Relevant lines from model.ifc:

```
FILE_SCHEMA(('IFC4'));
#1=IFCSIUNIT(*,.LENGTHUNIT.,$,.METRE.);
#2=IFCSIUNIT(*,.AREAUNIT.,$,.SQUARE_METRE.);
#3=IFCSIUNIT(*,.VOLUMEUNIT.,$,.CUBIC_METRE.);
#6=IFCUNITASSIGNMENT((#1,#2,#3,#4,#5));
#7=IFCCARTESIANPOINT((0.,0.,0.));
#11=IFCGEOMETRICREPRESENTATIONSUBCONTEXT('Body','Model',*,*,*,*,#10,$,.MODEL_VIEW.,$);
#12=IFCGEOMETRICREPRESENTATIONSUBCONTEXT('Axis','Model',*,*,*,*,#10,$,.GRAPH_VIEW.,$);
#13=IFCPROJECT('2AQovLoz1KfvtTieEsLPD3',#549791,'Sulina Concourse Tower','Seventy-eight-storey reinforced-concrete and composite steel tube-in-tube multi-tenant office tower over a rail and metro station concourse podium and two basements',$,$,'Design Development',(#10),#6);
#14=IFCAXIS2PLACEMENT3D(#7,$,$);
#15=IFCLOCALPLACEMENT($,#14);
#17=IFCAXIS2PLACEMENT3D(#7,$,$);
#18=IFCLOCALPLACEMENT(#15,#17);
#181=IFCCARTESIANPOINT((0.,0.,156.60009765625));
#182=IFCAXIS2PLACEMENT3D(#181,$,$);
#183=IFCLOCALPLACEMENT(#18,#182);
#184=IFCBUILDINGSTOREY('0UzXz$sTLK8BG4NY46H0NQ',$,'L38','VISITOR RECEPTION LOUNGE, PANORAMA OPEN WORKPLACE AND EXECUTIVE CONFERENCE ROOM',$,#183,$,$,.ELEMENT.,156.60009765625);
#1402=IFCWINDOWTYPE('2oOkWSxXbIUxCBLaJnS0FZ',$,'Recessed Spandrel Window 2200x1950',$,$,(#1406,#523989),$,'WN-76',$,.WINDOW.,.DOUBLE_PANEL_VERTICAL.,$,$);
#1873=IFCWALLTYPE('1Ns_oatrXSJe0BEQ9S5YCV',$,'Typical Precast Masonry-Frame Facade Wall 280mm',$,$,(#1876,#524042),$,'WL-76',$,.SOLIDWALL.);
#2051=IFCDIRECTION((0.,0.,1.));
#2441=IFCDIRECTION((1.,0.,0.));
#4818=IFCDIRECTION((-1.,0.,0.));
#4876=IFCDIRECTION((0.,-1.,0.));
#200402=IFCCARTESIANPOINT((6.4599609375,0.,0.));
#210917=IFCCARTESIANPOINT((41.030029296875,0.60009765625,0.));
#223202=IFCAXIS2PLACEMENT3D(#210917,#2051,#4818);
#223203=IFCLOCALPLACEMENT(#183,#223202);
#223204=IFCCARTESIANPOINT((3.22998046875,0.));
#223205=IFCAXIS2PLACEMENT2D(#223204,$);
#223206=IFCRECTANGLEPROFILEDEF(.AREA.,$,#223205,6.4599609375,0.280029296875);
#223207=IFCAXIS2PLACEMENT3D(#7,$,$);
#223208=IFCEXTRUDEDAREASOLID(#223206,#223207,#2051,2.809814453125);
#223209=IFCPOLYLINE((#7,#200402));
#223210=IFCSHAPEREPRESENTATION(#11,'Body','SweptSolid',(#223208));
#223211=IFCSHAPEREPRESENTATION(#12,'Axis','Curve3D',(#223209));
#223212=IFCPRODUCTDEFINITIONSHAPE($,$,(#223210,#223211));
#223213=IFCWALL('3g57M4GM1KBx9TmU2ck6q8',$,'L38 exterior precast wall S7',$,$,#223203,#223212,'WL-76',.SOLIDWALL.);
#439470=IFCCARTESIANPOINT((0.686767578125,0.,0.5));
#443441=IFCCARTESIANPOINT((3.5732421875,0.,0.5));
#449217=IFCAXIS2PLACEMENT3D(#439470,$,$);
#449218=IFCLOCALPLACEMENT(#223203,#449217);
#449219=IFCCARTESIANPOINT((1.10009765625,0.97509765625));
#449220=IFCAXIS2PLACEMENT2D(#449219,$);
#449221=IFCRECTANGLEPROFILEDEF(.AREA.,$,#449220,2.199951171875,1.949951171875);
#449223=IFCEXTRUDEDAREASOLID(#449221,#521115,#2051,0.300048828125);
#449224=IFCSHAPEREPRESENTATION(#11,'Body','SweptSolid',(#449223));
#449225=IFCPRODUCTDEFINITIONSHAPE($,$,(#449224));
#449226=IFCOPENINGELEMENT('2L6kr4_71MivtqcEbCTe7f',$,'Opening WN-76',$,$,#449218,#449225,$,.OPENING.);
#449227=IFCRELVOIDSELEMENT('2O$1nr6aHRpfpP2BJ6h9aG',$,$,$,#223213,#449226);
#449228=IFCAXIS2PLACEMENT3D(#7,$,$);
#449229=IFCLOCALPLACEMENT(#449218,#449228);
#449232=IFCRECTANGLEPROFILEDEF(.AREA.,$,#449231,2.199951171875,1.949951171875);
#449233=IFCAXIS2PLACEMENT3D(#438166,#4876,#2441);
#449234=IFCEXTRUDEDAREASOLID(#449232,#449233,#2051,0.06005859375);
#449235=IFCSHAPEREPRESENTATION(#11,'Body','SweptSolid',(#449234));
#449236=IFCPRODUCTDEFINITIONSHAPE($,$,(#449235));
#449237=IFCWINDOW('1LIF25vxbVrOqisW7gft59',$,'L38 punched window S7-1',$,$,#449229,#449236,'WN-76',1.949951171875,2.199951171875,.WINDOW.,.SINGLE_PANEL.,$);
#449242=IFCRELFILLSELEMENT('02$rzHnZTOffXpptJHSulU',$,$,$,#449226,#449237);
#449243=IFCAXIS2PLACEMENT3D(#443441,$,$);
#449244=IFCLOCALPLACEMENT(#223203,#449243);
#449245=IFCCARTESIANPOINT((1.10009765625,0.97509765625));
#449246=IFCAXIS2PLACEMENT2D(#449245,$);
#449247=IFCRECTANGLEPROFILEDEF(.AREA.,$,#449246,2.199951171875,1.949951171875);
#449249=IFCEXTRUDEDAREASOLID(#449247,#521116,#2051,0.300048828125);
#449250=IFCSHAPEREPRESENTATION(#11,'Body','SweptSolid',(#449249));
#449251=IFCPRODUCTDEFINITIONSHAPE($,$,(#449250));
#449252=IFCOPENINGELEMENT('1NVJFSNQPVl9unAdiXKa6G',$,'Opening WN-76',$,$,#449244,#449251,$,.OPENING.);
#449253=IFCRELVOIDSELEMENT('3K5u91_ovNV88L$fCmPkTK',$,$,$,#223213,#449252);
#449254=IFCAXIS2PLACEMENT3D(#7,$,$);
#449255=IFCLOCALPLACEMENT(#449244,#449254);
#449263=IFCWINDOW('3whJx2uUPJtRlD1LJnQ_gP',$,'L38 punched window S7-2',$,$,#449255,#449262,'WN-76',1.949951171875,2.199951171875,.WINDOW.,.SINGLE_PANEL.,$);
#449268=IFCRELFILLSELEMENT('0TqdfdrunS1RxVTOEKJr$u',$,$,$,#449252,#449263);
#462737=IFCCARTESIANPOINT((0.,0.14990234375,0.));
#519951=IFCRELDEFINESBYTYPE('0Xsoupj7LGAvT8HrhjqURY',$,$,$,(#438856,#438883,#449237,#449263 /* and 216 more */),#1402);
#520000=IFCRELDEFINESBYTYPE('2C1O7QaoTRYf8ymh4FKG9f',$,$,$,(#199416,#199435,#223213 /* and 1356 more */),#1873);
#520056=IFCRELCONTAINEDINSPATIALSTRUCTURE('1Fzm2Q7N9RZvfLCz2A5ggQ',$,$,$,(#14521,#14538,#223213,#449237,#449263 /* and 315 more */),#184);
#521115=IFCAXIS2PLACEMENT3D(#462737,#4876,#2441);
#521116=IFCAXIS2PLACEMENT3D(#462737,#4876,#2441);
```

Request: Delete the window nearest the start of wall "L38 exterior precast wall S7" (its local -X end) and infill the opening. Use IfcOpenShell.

```python
import ifcopenshell
import ifcopenshell.api.feature
import ifcopenshell.api.root
import ifcopenshell.geom
import ifcopenshell.util.shape

model = ifcopenshell.open("model.ifc")
settings = ifcopenshell.geom.settings()


def volume(element):
    """Net volume in cubic metres, openings subtracted."""
    shape = ifcopenshell.geom.create_shape(settings, element)
    return ifcopenshell.util.shape.get_volume(shape.geometry)


window = model.by_id(449237)
opening = window.FillsVoids[0].RelatingOpeningElement
wall = opening.VoidsElements[0].RelatingBuildingElement
before = volume(wall)

ifcopenshell.api.root.remove_product(model, product=window)
ifcopenshell.api.feature.remove_feature(model, feature=opening)

after = volume(wall)

print(f"wall volume {before:.3f} -> {after:.3f} m3")

model.write("model_v2.ifc")
```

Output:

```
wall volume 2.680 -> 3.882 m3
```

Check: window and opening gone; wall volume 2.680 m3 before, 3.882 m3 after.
